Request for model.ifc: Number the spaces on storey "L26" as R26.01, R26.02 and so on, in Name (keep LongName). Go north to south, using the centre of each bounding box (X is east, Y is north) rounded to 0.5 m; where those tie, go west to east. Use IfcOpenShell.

First a look at what the model holds.

```python
import ifcopenshell
import ifcopenshell.util.element
import ifcopenshell.util.placement

model = ifcopenshell.open("model.ifc")
print(model.schema)
storey = next(s for s in model.by_type("IfcBuildingStorey") if s.Name == "L26")
spaces = [e for e in ifcopenshell.util.element.get_decomposition(storey) if e.is_a("IfcSpace")]
for e in sorted(spaces, key=lambda e: e.id()):
    origin = ifcopenshell.util.placement.get_local_placement(e.ObjectPlacement)[:3, 3]
    print(e.id(), e.Name, e.LongName, origin.round(2) + 0.0, sep=" | ")
```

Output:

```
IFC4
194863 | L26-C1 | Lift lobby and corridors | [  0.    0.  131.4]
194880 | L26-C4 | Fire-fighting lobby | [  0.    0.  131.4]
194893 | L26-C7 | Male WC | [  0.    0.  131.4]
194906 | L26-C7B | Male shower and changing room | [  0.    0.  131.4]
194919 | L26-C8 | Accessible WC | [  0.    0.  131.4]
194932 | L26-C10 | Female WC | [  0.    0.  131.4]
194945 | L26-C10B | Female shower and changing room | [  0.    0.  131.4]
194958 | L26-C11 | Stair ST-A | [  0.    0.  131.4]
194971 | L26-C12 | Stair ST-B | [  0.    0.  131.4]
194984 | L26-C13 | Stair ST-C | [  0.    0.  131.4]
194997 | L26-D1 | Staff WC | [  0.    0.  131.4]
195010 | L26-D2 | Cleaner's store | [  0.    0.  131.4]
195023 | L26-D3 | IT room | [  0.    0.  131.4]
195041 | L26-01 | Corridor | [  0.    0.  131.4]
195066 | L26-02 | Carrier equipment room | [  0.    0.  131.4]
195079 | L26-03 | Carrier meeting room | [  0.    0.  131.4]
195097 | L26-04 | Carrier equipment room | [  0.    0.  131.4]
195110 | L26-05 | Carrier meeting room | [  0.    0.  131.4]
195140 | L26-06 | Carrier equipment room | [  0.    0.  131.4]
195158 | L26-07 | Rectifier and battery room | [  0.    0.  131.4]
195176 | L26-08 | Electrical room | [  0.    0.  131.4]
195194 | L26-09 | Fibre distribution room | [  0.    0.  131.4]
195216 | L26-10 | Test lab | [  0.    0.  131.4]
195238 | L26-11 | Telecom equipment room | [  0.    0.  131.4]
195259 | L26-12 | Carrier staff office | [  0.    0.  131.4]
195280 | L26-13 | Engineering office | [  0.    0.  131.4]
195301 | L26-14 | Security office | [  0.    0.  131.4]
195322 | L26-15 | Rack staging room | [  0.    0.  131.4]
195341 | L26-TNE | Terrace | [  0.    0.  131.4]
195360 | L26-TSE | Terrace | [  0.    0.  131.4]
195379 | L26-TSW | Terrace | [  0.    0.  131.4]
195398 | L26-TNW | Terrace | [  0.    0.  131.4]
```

```python
import ifcopenshell
import ifcopenshell.geom
import ifcopenshell.util.element
import ifcopenshell.util.shape

model = ifcopenshell.open("model.ifc")
settings = ifcopenshell.geom.settings()
settings.set("use-world-coords", True)


def centre(element):
    shape = ifcopenshell.geom.create_shape(settings, element)
    return ifcopenshell.util.shape.get_bbox_centroid(shape.geometry)


storey = next(s for s in model.by_type("IfcBuildingStorey") if s.Name == "L26")
spaces = [e for e in ifcopenshell.util.element.get_decomposition(storey) if e.is_a("IfcSpace")]

# Insertion points can sit at a corner or the storey origin, so sort by the geometry (in metres).
centres = {e: centre(e) for e in spaces}
spaces.sort(key=lambda e: (-round(centres[e][1] / 0.5), centres[e][0]))

for i, e in enumerate(spaces, start=1):
    number = f"R26.{i:02d}"
    e.Name = number
    print(e.id(), number)

model.write("model_rev.ifc")
```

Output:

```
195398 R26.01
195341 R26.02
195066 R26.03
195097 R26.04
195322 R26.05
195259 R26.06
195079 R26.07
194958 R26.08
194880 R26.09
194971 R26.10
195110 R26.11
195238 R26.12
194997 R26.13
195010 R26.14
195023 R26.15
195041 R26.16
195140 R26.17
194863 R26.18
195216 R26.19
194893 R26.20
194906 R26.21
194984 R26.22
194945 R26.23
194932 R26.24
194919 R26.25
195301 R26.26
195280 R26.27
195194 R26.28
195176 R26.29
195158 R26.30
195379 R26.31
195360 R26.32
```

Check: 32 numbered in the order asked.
